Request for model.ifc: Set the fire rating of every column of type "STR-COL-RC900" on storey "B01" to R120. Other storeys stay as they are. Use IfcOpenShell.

First a look at what the model holds.

```python
import ifcopenshell
import ifcopenshell.util.element

model = ifcopenshell.open("model.ifc")
print(model.schema)
storey = next(s for s in model.by_type("IfcBuildingStorey") if s.Name == "B01")
columns = [e for e in ifcopenshell.util.element.get_decomposition(storey) if e.is_a("IfcColumn")]
seen = {}
for e in columns:
    element_type = ifcopenshell.util.element.get_type(e)
    key = (element_type.Name if element_type != e and element_type else None, ifcopenshell.util.element.get_pset(e, "Pset_ColumnCommon", "FireRating"))
    seen[key] = seen.get(key, 0) + 1
for (name, value), count in sorted(seen.items(), key=str):
    print(count, "x", name, "|", value)
```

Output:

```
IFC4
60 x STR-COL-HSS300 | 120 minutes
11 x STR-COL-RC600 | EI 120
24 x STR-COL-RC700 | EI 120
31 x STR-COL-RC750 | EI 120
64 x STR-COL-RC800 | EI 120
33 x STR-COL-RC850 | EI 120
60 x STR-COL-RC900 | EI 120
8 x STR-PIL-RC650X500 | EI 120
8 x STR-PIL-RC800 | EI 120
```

```python
import ifcopenshell
import ifcopenshell.api.pset
import ifcopenshell.util.element

model = ifcopenshell.open("model.ifc")

storey = next(s for s in model.by_type("IfcBuildingStorey") if s.Name == "B01")
columns = [e for e in ifcopenshell.util.element.get_decomposition(storey) if e.is_a("IfcColumn")]

count = 0
for e in columns:
    element_type = ifcopenshell.util.element.get_type(e)
    if element_type in (None, e) or element_type.Name != "STR-COL-RC900":
        continue
    # add_pset returns the element's existing set when there is one.
    pset = ifcopenshell.api.pset.add_pset(model, product=e, name="Pset_ColumnCommon")
    ifcopenshell.api.pset.edit_pset(model, pset=pset, properties={"FireRating": "R120"})
    count += 1

print(count, "columns updated")

model.write("model_v2.ifc")
```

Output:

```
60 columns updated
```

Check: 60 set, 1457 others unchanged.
